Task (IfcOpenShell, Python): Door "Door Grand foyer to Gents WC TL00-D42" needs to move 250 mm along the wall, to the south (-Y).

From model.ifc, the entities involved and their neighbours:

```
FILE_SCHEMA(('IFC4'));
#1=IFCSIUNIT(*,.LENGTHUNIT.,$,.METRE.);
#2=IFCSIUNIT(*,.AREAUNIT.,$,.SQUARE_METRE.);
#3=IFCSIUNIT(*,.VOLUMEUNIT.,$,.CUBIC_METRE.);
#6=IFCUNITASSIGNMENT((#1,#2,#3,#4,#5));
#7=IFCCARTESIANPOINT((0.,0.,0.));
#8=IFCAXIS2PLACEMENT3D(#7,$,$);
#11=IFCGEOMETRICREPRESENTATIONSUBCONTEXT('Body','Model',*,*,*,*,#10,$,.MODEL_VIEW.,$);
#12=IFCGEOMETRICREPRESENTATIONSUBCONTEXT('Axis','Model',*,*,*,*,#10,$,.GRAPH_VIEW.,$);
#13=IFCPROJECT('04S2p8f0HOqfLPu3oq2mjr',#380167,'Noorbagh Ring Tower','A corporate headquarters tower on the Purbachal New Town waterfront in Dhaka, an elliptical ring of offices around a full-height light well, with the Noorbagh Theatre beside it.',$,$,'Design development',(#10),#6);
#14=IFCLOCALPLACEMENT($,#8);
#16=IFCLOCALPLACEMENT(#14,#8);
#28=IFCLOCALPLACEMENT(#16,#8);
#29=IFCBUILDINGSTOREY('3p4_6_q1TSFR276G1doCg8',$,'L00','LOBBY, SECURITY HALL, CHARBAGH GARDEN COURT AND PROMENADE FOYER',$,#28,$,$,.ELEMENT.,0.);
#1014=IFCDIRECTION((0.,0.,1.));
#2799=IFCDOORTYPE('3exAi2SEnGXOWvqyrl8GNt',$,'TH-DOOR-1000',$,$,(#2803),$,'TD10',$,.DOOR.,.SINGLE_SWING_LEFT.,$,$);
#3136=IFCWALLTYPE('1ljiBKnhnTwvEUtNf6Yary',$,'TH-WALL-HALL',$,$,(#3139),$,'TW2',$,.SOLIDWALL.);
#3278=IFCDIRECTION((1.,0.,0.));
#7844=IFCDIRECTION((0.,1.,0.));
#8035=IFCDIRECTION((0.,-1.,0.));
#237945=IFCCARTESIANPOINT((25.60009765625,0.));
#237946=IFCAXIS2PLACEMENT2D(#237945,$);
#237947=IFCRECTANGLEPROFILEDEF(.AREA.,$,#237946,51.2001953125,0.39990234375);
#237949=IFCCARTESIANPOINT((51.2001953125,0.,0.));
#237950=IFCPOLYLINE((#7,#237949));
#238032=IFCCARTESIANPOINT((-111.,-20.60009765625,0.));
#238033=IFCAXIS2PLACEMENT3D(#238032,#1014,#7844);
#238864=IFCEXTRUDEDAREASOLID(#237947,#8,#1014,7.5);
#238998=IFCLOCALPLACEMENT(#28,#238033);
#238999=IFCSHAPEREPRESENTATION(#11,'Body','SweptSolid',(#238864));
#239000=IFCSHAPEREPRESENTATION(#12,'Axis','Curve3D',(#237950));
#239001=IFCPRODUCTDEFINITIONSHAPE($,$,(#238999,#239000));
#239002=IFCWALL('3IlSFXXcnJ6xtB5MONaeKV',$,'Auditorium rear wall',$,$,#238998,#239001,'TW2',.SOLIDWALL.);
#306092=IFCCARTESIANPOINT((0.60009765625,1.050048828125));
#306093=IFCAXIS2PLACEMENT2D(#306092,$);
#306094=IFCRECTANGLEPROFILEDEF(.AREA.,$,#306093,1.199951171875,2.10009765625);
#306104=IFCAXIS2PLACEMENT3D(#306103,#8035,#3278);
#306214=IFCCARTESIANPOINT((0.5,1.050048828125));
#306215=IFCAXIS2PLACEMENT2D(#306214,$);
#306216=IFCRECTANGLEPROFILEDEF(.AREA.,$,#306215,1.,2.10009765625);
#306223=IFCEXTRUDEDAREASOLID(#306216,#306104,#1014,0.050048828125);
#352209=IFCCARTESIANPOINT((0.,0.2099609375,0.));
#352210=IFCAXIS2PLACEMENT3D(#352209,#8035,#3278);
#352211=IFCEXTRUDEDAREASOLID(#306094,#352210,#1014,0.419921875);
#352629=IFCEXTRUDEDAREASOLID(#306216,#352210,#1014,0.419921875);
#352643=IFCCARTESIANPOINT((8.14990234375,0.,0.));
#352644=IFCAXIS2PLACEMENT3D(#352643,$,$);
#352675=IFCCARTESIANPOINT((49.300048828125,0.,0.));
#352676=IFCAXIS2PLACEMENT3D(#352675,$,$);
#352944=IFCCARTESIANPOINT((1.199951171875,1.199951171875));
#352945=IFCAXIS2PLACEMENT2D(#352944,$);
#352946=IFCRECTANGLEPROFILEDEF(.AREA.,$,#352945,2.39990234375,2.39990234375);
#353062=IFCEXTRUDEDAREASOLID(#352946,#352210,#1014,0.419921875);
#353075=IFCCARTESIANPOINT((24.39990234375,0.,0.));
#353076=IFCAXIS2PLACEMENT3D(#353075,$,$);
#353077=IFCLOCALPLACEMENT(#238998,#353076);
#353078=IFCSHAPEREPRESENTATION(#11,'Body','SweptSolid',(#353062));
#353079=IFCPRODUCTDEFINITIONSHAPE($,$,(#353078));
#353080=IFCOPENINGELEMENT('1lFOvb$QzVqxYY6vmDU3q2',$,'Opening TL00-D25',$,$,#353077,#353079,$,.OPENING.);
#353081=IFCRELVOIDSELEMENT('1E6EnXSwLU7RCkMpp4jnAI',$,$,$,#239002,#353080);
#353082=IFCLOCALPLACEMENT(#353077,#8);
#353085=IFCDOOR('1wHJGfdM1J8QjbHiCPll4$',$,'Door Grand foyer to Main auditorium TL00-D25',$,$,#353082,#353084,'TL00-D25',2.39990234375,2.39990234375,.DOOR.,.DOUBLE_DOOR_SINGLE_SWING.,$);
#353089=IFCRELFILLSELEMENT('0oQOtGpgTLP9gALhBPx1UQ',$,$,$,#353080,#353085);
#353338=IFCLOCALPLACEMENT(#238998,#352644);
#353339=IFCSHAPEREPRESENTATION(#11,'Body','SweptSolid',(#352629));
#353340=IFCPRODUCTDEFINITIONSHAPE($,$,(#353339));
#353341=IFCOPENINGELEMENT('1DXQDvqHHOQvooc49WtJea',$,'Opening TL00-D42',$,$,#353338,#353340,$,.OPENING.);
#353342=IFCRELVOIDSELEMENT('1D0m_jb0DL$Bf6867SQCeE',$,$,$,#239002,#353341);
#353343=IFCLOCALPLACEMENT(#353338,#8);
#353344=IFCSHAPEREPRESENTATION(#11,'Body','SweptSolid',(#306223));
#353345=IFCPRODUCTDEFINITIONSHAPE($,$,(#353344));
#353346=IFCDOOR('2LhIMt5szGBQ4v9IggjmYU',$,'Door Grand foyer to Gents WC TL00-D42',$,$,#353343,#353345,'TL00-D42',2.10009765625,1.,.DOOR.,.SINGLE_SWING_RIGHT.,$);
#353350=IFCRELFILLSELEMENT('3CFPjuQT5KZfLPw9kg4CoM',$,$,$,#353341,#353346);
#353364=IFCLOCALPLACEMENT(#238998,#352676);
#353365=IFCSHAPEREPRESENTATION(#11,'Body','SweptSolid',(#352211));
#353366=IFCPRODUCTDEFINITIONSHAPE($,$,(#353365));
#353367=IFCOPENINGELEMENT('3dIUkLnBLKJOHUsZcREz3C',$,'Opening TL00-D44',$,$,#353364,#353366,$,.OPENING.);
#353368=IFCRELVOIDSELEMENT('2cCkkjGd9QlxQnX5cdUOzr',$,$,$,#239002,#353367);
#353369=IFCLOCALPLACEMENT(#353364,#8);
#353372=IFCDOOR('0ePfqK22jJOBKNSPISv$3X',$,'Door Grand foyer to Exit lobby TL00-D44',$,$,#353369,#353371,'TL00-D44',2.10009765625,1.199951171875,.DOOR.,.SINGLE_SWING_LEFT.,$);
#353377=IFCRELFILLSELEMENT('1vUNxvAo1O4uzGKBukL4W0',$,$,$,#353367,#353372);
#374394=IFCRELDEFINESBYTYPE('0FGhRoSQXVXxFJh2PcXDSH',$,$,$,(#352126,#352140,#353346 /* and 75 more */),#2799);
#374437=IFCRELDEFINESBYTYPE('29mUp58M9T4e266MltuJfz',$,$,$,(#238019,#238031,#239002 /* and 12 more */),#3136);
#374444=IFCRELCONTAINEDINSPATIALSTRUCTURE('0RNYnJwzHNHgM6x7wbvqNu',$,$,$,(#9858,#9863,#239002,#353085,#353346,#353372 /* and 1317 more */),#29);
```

```python
import ifcopenshell
import ifcopenshell.api.geometry
import ifcopenshell.util.placement

model = ifcopenshell.open("model.ifc")

door = model.by_id(353346)
opening = door.FillsVoids[0].RelatingOpeningElement
wall = opening.VoidsElements[0].RelatingBuildingElement

wall_matrix = ifcopenshell.util.placement.get_local_placement(wall.ObjectPlacement)
shift = wall_matrix[:3, 0] * -0.25
before = ifcopenshell.util.placement.get_local_placement(door.ObjectPlacement)[:3, 3].copy()

# The door is placed relative to its opening, so it follows when the opening moves.
matrix = ifcopenshell.util.placement.get_local_placement(opening.ObjectPlacement)
matrix[:3, 3] += shift
ifcopenshell.api.geometry.edit_object_placement(
    model, product=opening, matrix=matrix, is_si=False, should_transform_children=True
)

after = ifcopenshell.util.placement.get_local_placement(door.ObjectPlacement)[:3, 3]
print("door moved by", (after - before).round(3) + 0.0)

model.write("model-out.ifc")
```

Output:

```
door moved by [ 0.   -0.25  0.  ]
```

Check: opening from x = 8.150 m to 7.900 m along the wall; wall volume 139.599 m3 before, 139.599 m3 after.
